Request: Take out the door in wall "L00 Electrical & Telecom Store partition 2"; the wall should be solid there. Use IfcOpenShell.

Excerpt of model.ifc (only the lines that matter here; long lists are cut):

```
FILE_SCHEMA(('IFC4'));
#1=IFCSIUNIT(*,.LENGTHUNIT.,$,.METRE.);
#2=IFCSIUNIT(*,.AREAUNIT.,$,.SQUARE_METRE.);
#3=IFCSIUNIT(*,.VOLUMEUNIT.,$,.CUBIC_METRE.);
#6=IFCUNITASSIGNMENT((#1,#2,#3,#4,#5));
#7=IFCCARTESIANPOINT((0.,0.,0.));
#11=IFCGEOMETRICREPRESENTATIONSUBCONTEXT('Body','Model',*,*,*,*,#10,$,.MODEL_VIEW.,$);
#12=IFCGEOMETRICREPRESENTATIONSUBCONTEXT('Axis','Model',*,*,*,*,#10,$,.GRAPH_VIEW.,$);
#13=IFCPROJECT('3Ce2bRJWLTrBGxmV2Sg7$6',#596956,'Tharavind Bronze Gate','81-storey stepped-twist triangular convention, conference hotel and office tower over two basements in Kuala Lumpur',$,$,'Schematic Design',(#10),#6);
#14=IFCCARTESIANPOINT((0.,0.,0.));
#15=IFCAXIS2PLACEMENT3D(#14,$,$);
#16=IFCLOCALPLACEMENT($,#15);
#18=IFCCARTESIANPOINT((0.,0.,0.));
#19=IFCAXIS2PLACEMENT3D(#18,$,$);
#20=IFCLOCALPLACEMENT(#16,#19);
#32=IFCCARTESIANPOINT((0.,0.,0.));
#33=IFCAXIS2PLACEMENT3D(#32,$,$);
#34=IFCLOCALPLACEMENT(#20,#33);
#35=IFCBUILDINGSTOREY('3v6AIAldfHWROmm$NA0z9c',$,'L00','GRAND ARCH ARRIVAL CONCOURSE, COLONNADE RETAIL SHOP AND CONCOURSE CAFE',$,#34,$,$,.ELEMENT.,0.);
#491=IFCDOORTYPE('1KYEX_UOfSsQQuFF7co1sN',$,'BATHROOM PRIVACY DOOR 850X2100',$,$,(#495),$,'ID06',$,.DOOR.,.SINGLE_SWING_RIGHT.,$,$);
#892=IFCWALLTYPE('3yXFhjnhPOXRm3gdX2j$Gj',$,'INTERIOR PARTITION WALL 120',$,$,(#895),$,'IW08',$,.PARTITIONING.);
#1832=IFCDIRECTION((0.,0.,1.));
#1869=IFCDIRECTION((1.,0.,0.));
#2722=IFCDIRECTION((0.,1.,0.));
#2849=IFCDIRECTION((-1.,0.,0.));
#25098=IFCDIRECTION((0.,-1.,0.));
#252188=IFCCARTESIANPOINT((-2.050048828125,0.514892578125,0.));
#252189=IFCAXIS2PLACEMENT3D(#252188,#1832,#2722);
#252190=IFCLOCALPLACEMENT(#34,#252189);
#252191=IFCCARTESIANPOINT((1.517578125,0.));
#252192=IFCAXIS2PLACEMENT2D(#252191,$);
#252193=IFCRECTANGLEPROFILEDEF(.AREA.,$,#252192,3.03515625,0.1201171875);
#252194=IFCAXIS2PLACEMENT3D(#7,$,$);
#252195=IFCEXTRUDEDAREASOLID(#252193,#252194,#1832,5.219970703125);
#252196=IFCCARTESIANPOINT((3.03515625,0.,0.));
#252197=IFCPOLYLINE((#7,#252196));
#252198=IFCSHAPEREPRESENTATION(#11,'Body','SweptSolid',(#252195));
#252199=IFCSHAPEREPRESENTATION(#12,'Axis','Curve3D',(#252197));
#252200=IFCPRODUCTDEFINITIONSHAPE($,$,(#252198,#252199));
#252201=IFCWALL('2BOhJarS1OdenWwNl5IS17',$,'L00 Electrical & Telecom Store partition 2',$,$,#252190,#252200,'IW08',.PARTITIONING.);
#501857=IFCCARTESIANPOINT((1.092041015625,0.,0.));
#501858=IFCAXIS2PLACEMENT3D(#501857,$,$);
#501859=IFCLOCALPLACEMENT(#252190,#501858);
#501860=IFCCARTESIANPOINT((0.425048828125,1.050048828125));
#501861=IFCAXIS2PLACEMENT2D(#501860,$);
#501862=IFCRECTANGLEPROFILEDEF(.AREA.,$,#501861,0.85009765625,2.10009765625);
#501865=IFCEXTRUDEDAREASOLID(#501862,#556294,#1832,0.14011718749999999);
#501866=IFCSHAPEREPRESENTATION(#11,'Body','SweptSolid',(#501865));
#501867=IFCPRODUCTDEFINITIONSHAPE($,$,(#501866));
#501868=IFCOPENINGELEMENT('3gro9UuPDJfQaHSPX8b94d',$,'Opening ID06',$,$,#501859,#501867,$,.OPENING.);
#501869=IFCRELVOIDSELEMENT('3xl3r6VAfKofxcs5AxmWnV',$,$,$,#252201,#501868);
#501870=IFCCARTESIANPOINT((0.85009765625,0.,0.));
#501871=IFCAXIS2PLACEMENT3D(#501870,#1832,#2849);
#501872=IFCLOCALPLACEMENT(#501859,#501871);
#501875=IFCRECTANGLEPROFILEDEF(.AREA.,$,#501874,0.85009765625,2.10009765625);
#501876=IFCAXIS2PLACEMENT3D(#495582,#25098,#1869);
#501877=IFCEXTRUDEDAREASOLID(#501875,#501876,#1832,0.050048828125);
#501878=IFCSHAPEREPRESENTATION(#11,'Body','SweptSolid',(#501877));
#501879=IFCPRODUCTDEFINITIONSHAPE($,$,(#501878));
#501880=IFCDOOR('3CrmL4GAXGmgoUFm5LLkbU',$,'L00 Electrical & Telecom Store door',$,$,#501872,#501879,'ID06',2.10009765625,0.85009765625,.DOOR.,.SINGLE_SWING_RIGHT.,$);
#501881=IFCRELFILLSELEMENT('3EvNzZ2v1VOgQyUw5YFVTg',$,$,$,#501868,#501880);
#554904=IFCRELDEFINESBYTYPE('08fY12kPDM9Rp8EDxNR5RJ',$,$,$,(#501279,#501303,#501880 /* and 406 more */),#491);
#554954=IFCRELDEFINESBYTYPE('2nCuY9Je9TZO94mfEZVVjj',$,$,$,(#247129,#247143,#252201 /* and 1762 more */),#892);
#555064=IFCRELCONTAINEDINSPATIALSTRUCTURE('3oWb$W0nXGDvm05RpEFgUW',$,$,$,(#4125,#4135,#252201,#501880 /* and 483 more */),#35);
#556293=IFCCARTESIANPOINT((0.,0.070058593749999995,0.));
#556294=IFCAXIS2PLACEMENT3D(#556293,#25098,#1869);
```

```python
import ifcopenshell
import ifcopenshell.api.feature
import ifcopenshell.api.root
import ifcopenshell.geom
import ifcopenshell.util.shape

model = ifcopenshell.open("model.ifc")
settings = ifcopenshell.geom.settings()


def volume(element):
    """Net volume in cubic metres, openings subtracted."""
    shape = ifcopenshell.geom.create_shape(settings, element)
    return ifcopenshell.util.shape.get_volume(shape.geometry)


door = model.by_id(501880)
opening = door.FillsVoids[0].RelatingOpeningElement
wall = opening.VoidsElements[0].RelatingBuildingElement
before = volume(wall)

ifcopenshell.api.root.remove_product(model, product=door)
ifcopenshell.api.feature.remove_feature(model, feature=opening)

after = volume(wall)

print(f"wall volume {before:.3f} -> {after:.3f} m3")

model.write("model_edited.ifc")
```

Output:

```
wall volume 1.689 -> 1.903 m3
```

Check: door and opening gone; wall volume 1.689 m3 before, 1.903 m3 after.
